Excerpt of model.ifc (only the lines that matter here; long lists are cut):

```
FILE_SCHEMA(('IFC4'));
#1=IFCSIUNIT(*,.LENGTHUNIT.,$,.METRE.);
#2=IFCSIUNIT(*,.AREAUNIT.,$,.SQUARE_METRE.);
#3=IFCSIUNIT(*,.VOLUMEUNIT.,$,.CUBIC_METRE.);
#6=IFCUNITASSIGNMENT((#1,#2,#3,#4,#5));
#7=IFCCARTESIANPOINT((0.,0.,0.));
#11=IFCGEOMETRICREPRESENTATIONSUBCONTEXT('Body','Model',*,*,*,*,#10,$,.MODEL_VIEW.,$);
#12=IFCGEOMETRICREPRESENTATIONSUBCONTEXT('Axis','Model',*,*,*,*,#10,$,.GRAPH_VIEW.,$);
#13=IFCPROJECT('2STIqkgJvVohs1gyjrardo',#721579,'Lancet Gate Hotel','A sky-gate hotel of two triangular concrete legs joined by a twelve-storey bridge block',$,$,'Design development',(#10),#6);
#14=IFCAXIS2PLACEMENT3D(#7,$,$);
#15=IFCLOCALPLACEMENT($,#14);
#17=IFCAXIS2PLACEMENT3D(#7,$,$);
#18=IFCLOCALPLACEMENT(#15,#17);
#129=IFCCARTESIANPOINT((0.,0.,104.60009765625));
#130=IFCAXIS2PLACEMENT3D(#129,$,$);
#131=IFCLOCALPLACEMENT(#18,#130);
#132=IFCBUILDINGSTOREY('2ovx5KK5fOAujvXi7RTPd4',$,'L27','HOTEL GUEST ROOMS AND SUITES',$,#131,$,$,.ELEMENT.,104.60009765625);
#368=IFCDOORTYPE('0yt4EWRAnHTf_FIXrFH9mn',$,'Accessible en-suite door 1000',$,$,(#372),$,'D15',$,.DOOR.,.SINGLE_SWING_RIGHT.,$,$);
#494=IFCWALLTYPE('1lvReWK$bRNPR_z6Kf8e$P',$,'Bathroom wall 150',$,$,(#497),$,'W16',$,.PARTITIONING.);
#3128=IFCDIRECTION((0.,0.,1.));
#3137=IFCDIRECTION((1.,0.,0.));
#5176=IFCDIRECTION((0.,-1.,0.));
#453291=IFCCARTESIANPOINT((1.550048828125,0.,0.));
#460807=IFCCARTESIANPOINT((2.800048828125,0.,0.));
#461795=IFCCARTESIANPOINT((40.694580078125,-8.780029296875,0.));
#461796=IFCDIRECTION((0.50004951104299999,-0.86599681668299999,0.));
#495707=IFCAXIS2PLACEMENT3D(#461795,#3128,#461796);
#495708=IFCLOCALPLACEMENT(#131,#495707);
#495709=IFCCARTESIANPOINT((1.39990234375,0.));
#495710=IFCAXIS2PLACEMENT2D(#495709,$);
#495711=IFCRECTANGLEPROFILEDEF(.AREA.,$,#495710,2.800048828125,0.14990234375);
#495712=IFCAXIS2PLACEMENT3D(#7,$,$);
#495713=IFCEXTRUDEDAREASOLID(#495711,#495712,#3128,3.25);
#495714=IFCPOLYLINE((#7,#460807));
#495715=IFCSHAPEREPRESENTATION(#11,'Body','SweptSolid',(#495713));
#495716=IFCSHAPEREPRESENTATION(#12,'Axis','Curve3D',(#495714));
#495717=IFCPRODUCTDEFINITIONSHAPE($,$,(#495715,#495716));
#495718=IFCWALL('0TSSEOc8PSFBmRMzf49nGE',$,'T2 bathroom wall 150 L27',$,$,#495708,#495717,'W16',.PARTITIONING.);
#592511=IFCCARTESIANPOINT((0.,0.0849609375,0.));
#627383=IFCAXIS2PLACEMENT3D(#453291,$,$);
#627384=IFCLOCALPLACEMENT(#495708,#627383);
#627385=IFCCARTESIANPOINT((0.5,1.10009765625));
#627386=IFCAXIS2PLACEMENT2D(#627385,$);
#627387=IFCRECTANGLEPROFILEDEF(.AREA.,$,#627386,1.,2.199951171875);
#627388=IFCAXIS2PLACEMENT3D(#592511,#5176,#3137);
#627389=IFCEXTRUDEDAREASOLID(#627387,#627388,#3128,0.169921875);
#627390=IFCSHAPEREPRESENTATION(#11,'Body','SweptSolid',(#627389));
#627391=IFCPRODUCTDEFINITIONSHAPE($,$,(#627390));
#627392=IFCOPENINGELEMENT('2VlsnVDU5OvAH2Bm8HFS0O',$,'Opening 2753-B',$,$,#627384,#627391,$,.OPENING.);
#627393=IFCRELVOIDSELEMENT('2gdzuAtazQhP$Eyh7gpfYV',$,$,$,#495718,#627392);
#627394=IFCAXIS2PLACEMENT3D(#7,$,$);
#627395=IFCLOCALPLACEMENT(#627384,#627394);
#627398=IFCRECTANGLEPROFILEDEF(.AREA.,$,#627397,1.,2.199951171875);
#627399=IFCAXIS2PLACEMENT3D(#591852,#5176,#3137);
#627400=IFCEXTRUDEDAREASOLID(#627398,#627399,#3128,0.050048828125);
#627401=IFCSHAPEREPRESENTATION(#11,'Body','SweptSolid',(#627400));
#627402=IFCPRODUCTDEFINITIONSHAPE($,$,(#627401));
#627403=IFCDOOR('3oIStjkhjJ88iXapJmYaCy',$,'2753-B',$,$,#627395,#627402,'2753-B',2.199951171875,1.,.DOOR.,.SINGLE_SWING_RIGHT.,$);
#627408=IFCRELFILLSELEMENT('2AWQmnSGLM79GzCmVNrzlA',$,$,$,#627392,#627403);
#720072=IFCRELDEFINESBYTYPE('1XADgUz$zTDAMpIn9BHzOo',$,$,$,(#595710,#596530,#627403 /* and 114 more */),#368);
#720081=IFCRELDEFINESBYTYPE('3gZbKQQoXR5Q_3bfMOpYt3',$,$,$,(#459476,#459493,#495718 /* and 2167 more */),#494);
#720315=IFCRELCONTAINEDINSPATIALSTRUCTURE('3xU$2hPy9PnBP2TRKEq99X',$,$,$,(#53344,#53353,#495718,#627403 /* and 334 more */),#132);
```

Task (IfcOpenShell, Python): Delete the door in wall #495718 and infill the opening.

```python
import ifcopenshell
import ifcopenshell.api.feature
import ifcopenshell.api.root
import ifcopenshell.geom
import ifcopenshell.util.shape

model = ifcopenshell.open("model.ifc")
settings = ifcopenshell.geom.settings()


def volume(element):
    """Net volume in cubic metres, openings subtracted."""
    shape = ifcopenshell.geom.create_shape(settings, element)
    return ifcopenshell.util.shape.get_volume(shape.geometry)


door = model.by_guid("3oIStjkhjJ88iXapJmYaCy")
opening = door.FillsVoids[0].RelatingOpeningElement
wall = opening.VoidsElements[0].RelatingBuildingElement
before = volume(wall)

ifcopenshell.api.root.remove_product(model, product=door)
ifcopenshell.api.feature.remove_feature(model, feature=opening)

after = volume(wall)

print(f"wall volume {before:.3f} -> {after:.3f} m3")

model.write("model_updated.ifc")
```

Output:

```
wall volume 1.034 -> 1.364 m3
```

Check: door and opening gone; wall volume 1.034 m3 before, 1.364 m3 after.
